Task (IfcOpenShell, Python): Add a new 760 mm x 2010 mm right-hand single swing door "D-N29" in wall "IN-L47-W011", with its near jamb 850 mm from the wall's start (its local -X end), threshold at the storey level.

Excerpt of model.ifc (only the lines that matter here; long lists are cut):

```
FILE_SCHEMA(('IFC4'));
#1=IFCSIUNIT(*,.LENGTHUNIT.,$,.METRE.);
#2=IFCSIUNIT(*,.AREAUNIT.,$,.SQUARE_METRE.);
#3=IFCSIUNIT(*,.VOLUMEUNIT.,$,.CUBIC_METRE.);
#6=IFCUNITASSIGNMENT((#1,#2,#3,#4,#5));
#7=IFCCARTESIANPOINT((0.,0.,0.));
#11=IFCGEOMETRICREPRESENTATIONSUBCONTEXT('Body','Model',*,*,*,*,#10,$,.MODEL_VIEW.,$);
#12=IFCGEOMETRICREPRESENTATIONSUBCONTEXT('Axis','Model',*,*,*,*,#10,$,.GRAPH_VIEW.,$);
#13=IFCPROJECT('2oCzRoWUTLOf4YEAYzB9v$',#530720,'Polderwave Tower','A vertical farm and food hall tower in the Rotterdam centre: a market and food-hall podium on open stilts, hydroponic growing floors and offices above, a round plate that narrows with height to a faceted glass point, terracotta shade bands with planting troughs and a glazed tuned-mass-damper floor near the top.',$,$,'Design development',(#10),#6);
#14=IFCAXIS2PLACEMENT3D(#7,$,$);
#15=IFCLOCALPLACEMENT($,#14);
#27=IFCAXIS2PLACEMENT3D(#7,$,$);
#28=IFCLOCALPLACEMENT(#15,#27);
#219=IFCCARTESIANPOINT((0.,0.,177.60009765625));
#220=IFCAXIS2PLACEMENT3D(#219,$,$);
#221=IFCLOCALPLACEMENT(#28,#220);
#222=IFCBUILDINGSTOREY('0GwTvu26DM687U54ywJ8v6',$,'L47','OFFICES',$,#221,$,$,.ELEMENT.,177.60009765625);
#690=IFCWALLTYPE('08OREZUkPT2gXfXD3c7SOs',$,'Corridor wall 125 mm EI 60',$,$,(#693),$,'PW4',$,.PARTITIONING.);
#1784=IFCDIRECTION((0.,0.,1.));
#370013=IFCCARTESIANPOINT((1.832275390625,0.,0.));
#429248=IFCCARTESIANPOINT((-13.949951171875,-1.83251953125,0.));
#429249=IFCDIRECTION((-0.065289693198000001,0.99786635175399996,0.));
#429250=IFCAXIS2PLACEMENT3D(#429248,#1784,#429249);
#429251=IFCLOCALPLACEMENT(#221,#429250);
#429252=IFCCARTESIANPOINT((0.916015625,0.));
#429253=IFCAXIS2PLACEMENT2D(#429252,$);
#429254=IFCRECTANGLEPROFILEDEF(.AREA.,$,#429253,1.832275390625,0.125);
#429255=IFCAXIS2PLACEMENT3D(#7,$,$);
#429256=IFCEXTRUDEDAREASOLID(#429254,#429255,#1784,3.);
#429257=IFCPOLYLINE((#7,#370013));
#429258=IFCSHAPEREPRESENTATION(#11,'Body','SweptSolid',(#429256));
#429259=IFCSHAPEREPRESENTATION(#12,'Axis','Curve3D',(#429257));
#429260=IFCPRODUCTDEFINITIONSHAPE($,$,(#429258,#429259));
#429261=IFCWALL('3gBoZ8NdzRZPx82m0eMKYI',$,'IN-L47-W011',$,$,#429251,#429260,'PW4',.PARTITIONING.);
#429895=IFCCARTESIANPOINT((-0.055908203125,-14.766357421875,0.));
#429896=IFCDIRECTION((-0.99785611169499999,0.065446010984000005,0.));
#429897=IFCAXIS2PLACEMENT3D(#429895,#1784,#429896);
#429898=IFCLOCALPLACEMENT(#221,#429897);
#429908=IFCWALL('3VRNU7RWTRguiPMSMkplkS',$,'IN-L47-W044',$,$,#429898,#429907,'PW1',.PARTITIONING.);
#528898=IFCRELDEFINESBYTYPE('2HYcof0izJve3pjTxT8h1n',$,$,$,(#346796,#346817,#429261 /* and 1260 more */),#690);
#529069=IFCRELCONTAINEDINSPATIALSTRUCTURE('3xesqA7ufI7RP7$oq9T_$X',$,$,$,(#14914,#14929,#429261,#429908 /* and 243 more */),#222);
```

```python
import numpy as np
import ifcopenshell
import ifcopenshell.api.feature
import ifcopenshell.api.geometry
import ifcopenshell.api.root
import ifcopenshell.api.spatial
import ifcopenshell.geom
import ifcopenshell.util.element
import ifcopenshell.util.placement
import ifcopenshell.util.representation
import ifcopenshell.util.shape
import ifcopenshell.util.unit

model = ifcopenshell.open("model.ifc")
unit_scale = ifcopenshell.util.unit.calculate_unit_scale(model)
settings = ifcopenshell.geom.settings()


def volume(element):
    """Net volume in cubic metres, openings subtracted."""
    shape = ifcopenshell.geom.create_shape(settings, element)
    return ifcopenshell.util.shape.get_volume(shape.geometry)


wall = model.by_guid("3gBoZ8NdzRZPx82m0eMKYI")
storey = ifcopenshell.util.element.get_container(wall, ifc_class="IfcBuildingStorey")
context = ifcopenshell.util.representation.get_context(model, "Model", "Body", "MODEL_VIEW")
before = volume(wall)

width, height, from_end, sill = 0.76, 2.01, 0.85, 0.0  # metres

# The wall runs along its own X axis, and the end named is its -X end.
wall_shape = ifcopenshell.geom.create_shape(settings, wall)
x, y, z = ifcopenshell.util.shape.get_vertices(wall_shape.geometry).T
start = x.min() + from_end
face, thickness = float(y.min()), float(y.max() - y.min())
wall_matrix = ifcopenshell.util.placement.get_local_placement(wall.ObjectPlacement)
level = ifcopenshell.util.placement.get_local_placement(storey.ObjectPlacement)[2, 3]


def in_wall(x, y):
    """Placement at x, y metres in the wall's axes, at sill height."""
    matrix = wall_matrix.copy()
    matrix[:, 3] = wall_matrix @ np.array([x / unit_scale, y / unit_scale, 0.0, 1.0])
    matrix[2, 3] = level + sill / unit_scale
    return matrix


# Opening: a box that overshoots both wall faces by 50 mm.
opening = ifcopenshell.api.root.create_entity(model, ifc_class="IfcOpeningElement", predefined_type="OPENING")
box = ifcopenshell.api.geometry.add_wall_representation(
    model, context=context, length=width, height=height, thickness=thickness + 0.1
)
ifcopenshell.api.geometry.assign_representation(model, product=opening, representation=box)
ifcopenshell.api.geometry.edit_object_placement(model, product=opening, matrix=in_wall(start, face - 0.05), is_si=False)
ifcopenshell.api.feature.add_feature(model, feature=opening, element=wall)

door = ifcopenshell.api.root.create_entity(model, ifc_class="IfcDoor", name="D-N29", predefined_type="DOOR")
door.OverallWidth, door.OverallHeight = width / unit_scale, height / unit_scale
door.OperationType = "SINGLE_SWING_RIGHT"
body = ifcopenshell.api.geometry.add_door_representation(
    model,
    context=context,
    overall_width=door.OverallWidth,
    overall_height=door.OverallHeight,
    operation_type="SINGLE_SWING_RIGHT",
    lining_properties={"LiningDepth": thickness / unit_scale, "ThresholdDepth": thickness / unit_scale},
)
ifcopenshell.api.geometry.assign_representation(model, product=door, representation=body)
ifcopenshell.api.spatial.assign_container(model, products=[door], relating_structure=storey)
ifcopenshell.api.feature.add_filling(model, opening=opening, element=door)

# The lining spans the wall, so the door starts at the wall face.
ifcopenshell.api.geometry.edit_object_placement(model, product=door, matrix=in_wall(start, face), is_si=False)

after = volume(wall)

print(f"wall volume {before:.3f} -> {after:.3f} m3")

model.write("model_updated.ifc")
```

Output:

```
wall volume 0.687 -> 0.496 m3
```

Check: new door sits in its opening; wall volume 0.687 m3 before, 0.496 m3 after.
